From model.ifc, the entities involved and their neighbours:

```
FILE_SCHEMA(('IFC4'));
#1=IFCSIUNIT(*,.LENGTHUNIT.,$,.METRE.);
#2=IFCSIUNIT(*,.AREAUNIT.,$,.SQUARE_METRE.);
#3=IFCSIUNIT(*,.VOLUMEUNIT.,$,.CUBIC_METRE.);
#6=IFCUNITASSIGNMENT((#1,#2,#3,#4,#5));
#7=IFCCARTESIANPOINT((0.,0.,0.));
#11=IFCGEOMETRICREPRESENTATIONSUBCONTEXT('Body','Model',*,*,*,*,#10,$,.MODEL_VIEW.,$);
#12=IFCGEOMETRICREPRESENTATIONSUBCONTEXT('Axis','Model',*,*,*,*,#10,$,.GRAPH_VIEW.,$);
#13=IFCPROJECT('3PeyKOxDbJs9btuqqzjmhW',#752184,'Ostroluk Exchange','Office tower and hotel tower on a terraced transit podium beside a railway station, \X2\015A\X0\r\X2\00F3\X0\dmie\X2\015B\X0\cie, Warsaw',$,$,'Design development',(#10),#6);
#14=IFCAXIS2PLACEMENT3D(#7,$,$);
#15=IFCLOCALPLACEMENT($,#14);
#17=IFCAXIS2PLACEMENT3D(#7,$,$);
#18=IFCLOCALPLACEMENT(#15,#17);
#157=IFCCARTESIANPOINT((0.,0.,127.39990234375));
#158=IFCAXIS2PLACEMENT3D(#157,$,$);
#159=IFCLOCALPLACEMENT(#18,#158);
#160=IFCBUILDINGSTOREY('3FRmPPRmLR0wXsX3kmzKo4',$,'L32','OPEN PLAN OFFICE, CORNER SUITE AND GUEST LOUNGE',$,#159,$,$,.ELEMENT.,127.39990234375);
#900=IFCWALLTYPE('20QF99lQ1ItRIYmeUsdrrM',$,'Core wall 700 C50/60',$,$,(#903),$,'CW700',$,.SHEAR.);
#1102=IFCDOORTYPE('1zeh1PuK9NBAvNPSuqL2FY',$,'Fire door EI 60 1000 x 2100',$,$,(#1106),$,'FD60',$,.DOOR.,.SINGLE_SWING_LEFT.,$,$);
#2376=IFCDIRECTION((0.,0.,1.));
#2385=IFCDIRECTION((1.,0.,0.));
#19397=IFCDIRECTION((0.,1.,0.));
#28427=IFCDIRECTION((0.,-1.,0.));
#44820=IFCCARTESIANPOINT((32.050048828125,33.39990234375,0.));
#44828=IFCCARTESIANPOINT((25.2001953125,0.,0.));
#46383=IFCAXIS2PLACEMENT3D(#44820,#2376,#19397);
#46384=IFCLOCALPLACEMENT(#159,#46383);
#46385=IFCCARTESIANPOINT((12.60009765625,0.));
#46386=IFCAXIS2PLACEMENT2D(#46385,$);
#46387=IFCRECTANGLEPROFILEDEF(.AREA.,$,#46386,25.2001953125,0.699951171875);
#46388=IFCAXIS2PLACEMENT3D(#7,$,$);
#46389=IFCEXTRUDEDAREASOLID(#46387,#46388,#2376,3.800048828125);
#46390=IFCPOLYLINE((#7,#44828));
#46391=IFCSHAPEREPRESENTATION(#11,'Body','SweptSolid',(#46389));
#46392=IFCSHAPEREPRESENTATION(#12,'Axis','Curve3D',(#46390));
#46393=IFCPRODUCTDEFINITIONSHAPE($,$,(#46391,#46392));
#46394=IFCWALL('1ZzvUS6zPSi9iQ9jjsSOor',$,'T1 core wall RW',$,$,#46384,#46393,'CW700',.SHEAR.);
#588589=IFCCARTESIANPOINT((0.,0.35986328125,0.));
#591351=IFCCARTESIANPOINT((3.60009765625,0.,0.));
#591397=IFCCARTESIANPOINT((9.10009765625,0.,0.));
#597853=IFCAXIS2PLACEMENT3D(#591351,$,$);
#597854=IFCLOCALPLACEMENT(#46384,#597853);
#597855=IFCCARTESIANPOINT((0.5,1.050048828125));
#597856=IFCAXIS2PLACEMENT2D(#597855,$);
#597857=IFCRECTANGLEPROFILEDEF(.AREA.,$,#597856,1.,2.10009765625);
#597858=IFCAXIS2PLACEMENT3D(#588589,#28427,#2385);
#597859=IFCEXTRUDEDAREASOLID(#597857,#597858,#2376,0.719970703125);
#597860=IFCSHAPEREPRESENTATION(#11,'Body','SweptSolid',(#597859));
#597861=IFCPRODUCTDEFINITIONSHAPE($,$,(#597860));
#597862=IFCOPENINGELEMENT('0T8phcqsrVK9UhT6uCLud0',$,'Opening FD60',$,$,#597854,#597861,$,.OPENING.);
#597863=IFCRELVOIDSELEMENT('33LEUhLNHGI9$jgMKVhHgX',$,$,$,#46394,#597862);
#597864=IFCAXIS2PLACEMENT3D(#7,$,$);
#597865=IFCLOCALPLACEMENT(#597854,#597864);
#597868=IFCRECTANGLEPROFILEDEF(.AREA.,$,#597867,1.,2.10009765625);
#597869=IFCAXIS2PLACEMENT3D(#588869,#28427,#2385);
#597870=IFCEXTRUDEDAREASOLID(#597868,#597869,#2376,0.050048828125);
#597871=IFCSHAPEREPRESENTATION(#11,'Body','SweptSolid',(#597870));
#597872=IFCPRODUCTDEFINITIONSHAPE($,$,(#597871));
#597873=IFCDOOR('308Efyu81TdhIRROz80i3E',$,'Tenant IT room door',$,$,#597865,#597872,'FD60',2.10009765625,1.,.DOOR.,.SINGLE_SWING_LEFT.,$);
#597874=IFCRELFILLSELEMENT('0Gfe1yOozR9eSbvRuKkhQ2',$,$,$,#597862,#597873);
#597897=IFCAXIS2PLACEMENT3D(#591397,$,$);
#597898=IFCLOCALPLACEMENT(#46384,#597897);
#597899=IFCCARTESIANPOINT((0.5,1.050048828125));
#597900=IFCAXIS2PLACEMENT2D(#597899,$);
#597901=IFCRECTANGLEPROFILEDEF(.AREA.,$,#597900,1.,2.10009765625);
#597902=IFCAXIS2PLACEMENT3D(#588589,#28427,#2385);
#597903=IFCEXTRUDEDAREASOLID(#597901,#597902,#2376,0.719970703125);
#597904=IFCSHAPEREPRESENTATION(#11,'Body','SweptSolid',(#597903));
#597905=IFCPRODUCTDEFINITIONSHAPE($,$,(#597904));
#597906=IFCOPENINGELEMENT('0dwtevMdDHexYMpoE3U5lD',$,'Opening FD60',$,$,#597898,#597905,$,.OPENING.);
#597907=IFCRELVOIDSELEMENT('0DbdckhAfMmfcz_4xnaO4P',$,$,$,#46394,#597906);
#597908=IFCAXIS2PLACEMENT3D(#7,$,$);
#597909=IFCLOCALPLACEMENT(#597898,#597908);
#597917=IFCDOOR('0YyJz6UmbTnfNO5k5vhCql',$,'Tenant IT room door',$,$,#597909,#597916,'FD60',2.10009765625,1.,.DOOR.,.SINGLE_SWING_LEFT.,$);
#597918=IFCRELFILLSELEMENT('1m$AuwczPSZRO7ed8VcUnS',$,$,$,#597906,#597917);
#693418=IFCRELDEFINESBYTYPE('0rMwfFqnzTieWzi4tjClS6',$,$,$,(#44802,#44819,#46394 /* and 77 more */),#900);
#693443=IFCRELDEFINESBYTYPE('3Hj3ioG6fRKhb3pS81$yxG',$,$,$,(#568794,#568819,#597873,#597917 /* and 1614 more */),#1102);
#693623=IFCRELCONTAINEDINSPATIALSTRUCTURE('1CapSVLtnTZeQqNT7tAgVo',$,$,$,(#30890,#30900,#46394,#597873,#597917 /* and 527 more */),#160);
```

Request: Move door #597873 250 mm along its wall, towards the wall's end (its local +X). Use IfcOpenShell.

```python
import ifcopenshell
import ifcopenshell.api.geometry
import ifcopenshell.util.placement
import ifcopenshell.util.unit

model = ifcopenshell.open("model.ifc")
unit_scale = ifcopenshell.util.unit.calculate_unit_scale(model)

door = model.by_guid("308Efyu81TdhIRROz80i3E")
opening = door.FillsVoids[0].RelatingOpeningElement
wall = opening.VoidsElements[0].RelatingBuildingElement

wall_matrix = ifcopenshell.util.placement.get_local_placement(wall.ObjectPlacement)
shift = wall_matrix[:3, 0] * 0.25 / unit_scale
before = ifcopenshell.util.placement.get_local_placement(door.ObjectPlacement)[:3, 3].copy()

# The door is placed relative to its opening, so it follows when the opening moves.
matrix = ifcopenshell.util.placement.get_local_placement(opening.ObjectPlacement)
matrix[:3, 3] += shift
ifcopenshell.api.geometry.edit_object_placement(
    model, product=opening, matrix=matrix, is_si=False, should_transform_children=True
)

after = ifcopenshell.util.placement.get_local_placement(door.ObjectPlacement)[:3, 3]
print("door moved by", (after - before).round(3) + 0.0)

model.write("model-out.ifc")
```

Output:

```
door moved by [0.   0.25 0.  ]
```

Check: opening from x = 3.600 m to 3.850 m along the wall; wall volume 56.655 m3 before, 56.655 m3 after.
